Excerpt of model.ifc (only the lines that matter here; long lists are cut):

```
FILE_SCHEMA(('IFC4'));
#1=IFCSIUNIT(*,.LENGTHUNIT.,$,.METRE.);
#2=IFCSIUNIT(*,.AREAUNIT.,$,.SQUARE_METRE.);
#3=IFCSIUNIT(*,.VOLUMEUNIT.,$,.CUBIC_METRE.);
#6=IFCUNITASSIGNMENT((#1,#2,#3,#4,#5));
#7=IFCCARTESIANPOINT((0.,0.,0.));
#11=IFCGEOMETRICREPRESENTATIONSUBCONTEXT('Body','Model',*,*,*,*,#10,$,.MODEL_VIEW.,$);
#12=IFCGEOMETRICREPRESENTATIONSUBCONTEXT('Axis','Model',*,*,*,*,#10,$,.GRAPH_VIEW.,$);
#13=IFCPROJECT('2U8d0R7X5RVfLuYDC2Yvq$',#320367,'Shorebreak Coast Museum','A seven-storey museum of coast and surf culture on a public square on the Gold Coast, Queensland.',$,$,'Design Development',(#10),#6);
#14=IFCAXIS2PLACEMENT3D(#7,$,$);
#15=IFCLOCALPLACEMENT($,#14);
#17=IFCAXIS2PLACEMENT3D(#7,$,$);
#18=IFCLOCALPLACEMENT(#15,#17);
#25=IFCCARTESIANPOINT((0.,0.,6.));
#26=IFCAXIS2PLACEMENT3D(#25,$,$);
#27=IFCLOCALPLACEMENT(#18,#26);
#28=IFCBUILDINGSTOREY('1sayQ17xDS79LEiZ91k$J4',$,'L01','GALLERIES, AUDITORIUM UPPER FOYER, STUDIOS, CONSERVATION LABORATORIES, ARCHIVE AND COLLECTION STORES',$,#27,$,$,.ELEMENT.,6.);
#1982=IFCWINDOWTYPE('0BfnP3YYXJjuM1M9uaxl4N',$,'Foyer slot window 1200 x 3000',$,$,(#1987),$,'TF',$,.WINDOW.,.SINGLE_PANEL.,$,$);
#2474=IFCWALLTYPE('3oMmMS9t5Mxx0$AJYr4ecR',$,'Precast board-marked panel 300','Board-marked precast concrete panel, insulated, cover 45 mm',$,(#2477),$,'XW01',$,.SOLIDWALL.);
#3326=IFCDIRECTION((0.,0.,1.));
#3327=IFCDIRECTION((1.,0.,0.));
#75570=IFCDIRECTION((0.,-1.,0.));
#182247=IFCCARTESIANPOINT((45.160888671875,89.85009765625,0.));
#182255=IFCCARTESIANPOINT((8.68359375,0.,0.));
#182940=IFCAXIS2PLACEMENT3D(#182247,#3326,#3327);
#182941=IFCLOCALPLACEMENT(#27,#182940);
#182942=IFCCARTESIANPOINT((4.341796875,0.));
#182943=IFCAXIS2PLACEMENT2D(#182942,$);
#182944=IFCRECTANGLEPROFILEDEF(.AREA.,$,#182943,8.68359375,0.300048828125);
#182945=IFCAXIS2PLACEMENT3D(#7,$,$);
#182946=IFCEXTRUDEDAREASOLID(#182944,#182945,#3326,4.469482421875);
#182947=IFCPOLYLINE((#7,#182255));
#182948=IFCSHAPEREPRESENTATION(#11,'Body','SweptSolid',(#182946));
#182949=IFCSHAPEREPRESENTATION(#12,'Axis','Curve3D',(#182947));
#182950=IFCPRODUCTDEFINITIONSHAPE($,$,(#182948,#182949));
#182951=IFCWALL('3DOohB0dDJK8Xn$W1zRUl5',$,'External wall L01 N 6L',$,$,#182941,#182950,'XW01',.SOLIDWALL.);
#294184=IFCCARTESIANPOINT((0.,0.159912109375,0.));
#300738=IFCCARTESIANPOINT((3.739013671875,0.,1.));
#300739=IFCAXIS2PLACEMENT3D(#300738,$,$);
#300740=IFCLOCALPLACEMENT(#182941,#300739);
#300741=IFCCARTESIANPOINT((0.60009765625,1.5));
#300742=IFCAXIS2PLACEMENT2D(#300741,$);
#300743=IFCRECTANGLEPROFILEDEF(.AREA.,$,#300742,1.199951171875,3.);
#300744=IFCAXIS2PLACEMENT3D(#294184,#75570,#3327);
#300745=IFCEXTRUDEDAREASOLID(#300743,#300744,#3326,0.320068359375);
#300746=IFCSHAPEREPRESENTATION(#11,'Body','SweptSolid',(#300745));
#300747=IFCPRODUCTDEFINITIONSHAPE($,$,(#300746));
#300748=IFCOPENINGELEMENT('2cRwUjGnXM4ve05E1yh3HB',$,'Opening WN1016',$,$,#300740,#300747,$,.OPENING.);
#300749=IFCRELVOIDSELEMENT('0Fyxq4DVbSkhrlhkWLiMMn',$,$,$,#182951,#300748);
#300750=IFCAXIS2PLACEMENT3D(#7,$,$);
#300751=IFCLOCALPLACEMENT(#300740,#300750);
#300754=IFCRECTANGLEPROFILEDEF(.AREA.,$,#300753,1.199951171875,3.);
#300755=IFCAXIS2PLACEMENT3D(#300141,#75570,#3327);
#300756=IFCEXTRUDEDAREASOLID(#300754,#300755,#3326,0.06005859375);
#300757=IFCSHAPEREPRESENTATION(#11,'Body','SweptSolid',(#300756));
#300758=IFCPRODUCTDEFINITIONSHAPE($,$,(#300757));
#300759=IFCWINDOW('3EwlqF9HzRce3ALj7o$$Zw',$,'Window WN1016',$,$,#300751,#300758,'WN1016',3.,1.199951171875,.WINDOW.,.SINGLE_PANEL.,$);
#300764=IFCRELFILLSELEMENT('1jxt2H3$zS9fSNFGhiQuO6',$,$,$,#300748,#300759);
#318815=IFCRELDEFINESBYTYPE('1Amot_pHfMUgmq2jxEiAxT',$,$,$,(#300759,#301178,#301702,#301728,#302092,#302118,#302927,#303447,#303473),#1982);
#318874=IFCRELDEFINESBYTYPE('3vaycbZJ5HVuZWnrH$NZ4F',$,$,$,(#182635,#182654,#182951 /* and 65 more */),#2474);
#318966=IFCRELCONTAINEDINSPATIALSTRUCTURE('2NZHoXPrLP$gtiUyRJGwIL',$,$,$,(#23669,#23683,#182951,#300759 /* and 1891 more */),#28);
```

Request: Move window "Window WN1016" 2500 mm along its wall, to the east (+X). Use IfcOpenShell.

```python
import ifcopenshell
import ifcopenshell.api.geometry
import ifcopenshell.util.placement
import ifcopenshell.util.unit

model = ifcopenshell.open("model.ifc")
unit_scale = ifcopenshell.util.unit.calculate_unit_scale(model)

window = model.by_guid("3EwlqF9HzRce3ALj7o$$Zw")
opening = window.FillsVoids[0].RelatingOpeningElement
wall = opening.VoidsElements[0].RelatingBuildingElement

wall_matrix = ifcopenshell.util.placement.get_local_placement(wall.ObjectPlacement)
shift = wall_matrix[:3, 0] * 2.5 / unit_scale
before = ifcopenshell.util.placement.get_local_placement(window.ObjectPlacement)[:3, 3].copy()

# The window is placed relative to its opening, so it follows when the opening moves.
matrix = ifcopenshell.util.placement.get_local_placement(opening.ObjectPlacement)
matrix[:3, 3] += shift
ifcopenshell.api.geometry.edit_object_placement(
    model, product=opening, matrix=matrix, is_si=False, should_transform_children=True
)

after = ifcopenshell.util.placement.get_local_placement(window.ObjectPlacement)[:3, 3]
print("window moved by", (after - before).round(3) + 0.0)

model.write("model-out.ifc")
```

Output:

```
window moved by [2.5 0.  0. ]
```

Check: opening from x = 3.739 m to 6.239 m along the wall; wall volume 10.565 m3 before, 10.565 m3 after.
